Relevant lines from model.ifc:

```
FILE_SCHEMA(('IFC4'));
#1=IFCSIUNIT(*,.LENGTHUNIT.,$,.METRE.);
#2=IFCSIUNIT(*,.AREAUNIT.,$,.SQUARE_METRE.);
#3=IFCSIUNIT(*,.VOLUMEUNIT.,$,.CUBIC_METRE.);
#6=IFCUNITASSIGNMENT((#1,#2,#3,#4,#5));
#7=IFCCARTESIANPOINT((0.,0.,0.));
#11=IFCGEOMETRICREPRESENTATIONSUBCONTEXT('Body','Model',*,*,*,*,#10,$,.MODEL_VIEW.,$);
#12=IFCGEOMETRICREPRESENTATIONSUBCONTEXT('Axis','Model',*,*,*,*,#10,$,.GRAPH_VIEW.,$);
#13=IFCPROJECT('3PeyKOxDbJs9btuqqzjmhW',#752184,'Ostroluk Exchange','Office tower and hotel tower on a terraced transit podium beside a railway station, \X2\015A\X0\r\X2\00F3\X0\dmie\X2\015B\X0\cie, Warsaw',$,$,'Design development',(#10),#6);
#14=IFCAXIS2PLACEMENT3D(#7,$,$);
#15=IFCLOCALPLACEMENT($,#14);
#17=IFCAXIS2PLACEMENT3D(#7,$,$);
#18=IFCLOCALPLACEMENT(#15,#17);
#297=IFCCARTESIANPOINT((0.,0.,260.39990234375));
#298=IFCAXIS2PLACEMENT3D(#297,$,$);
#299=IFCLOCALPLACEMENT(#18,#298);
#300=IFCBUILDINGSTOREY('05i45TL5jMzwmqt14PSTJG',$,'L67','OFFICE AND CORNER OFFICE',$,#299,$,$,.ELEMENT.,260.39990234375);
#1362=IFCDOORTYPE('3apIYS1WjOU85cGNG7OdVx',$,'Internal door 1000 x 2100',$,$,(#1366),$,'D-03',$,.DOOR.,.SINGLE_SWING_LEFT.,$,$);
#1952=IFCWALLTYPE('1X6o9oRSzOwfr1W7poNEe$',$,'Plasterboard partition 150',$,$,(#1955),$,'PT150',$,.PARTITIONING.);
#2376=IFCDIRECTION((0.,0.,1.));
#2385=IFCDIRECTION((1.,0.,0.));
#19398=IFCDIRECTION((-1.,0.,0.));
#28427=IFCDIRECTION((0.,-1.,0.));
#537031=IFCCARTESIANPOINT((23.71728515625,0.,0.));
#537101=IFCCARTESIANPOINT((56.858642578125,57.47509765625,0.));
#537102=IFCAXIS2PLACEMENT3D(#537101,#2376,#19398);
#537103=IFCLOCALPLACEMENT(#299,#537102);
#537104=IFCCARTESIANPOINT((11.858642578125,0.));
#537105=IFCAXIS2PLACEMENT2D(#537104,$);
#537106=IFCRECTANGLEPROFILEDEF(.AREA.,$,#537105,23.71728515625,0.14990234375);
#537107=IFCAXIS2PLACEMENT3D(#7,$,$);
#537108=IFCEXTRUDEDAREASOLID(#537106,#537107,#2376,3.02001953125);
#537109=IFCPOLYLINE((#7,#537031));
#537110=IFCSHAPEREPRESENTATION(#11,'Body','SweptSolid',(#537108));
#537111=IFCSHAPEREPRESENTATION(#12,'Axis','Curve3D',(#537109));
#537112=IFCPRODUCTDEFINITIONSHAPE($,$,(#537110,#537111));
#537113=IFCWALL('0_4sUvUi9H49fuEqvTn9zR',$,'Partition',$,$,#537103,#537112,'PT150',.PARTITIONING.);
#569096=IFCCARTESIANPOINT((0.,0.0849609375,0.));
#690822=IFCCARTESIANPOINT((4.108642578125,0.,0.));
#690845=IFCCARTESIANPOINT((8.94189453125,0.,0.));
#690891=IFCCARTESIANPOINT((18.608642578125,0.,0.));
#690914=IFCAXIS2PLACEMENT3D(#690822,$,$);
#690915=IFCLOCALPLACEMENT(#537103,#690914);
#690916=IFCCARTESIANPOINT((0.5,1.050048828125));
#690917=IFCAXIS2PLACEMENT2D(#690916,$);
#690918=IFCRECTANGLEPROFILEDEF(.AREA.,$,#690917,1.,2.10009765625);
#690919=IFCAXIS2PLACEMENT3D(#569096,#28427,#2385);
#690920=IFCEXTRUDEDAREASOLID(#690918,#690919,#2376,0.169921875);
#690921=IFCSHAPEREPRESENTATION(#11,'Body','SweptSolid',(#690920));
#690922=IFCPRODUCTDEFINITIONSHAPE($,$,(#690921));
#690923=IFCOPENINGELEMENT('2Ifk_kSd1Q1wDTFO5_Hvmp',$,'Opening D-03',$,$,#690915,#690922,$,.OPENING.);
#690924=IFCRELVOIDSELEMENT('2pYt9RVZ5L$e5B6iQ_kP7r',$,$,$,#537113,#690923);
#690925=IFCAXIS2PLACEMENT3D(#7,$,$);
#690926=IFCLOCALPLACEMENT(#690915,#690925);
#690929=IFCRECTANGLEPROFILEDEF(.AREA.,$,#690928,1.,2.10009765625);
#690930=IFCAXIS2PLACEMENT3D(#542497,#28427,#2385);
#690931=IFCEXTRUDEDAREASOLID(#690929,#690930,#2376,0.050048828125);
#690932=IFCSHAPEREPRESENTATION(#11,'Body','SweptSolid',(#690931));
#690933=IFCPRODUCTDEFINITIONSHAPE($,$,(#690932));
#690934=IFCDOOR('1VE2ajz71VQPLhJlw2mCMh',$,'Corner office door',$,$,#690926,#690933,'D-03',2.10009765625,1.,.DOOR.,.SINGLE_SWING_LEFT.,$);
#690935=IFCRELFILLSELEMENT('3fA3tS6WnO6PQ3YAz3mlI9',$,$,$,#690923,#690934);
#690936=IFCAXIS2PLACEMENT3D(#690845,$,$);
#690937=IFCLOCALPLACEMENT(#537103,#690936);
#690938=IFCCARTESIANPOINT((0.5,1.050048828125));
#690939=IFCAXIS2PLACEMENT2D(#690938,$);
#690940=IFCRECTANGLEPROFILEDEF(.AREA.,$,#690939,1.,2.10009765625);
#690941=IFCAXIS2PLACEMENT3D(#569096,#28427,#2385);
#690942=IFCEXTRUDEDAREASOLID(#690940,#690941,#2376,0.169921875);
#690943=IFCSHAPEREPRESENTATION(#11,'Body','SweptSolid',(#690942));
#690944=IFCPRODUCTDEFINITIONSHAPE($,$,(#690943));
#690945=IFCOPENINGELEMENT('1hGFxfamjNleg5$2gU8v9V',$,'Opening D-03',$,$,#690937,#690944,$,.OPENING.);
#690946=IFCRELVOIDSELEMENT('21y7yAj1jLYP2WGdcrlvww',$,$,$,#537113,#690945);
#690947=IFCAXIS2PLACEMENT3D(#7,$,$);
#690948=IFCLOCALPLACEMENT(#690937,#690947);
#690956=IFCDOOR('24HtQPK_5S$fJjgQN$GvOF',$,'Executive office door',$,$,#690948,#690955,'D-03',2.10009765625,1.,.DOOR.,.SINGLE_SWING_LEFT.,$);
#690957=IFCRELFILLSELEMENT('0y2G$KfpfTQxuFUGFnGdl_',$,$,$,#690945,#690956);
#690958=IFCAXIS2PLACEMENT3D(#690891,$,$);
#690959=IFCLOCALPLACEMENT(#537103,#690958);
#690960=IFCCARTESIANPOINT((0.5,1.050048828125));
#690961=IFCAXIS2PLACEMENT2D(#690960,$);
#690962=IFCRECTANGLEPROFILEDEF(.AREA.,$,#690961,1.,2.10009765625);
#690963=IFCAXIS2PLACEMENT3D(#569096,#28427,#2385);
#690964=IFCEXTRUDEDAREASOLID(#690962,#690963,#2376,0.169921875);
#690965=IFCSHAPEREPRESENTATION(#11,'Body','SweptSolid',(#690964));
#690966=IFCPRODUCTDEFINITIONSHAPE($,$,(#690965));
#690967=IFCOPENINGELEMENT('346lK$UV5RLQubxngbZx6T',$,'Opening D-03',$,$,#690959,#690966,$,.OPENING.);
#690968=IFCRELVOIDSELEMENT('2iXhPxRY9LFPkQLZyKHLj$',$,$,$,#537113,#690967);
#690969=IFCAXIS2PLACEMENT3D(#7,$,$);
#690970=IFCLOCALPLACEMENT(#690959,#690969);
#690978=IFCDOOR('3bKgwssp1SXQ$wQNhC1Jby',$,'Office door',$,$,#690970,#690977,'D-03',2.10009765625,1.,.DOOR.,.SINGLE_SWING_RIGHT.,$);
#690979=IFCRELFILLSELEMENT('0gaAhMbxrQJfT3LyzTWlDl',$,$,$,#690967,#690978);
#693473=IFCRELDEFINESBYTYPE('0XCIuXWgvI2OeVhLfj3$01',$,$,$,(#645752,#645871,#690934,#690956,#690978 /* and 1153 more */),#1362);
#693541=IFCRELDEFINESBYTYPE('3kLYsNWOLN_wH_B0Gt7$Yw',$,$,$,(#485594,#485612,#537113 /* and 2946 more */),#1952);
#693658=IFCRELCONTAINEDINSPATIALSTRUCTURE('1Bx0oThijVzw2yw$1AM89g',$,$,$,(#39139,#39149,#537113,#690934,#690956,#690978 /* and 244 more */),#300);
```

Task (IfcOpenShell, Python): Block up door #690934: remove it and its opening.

```python
import ifcopenshell
import ifcopenshell.api.feature
import ifcopenshell.api.root
import ifcopenshell.geom
import ifcopenshell.util.shape

model = ifcopenshell.open("model.ifc")
settings = ifcopenshell.geom.settings()


def volume(element):
    """Net volume in cubic metres, openings subtracted."""
    shape = ifcopenshell.geom.create_shape(settings, element)
    return ifcopenshell.util.shape.get_volume(shape.geometry)


door = model.by_id(690934)
opening = door.FillsVoids[0].RelatingOpeningElement
wall = opening.VoidsElements[0].RelatingBuildingElement
before = volume(wall)

ifcopenshell.api.root.remove_product(model, product=door)
ifcopenshell.api.feature.remove_feature(model, feature=opening)

after = volume(wall)

print(f"wall volume {before:.3f} -> {after:.3f} m3")

model.write("model_edited.ifc")
```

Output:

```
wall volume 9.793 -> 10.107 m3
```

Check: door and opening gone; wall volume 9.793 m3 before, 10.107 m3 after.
